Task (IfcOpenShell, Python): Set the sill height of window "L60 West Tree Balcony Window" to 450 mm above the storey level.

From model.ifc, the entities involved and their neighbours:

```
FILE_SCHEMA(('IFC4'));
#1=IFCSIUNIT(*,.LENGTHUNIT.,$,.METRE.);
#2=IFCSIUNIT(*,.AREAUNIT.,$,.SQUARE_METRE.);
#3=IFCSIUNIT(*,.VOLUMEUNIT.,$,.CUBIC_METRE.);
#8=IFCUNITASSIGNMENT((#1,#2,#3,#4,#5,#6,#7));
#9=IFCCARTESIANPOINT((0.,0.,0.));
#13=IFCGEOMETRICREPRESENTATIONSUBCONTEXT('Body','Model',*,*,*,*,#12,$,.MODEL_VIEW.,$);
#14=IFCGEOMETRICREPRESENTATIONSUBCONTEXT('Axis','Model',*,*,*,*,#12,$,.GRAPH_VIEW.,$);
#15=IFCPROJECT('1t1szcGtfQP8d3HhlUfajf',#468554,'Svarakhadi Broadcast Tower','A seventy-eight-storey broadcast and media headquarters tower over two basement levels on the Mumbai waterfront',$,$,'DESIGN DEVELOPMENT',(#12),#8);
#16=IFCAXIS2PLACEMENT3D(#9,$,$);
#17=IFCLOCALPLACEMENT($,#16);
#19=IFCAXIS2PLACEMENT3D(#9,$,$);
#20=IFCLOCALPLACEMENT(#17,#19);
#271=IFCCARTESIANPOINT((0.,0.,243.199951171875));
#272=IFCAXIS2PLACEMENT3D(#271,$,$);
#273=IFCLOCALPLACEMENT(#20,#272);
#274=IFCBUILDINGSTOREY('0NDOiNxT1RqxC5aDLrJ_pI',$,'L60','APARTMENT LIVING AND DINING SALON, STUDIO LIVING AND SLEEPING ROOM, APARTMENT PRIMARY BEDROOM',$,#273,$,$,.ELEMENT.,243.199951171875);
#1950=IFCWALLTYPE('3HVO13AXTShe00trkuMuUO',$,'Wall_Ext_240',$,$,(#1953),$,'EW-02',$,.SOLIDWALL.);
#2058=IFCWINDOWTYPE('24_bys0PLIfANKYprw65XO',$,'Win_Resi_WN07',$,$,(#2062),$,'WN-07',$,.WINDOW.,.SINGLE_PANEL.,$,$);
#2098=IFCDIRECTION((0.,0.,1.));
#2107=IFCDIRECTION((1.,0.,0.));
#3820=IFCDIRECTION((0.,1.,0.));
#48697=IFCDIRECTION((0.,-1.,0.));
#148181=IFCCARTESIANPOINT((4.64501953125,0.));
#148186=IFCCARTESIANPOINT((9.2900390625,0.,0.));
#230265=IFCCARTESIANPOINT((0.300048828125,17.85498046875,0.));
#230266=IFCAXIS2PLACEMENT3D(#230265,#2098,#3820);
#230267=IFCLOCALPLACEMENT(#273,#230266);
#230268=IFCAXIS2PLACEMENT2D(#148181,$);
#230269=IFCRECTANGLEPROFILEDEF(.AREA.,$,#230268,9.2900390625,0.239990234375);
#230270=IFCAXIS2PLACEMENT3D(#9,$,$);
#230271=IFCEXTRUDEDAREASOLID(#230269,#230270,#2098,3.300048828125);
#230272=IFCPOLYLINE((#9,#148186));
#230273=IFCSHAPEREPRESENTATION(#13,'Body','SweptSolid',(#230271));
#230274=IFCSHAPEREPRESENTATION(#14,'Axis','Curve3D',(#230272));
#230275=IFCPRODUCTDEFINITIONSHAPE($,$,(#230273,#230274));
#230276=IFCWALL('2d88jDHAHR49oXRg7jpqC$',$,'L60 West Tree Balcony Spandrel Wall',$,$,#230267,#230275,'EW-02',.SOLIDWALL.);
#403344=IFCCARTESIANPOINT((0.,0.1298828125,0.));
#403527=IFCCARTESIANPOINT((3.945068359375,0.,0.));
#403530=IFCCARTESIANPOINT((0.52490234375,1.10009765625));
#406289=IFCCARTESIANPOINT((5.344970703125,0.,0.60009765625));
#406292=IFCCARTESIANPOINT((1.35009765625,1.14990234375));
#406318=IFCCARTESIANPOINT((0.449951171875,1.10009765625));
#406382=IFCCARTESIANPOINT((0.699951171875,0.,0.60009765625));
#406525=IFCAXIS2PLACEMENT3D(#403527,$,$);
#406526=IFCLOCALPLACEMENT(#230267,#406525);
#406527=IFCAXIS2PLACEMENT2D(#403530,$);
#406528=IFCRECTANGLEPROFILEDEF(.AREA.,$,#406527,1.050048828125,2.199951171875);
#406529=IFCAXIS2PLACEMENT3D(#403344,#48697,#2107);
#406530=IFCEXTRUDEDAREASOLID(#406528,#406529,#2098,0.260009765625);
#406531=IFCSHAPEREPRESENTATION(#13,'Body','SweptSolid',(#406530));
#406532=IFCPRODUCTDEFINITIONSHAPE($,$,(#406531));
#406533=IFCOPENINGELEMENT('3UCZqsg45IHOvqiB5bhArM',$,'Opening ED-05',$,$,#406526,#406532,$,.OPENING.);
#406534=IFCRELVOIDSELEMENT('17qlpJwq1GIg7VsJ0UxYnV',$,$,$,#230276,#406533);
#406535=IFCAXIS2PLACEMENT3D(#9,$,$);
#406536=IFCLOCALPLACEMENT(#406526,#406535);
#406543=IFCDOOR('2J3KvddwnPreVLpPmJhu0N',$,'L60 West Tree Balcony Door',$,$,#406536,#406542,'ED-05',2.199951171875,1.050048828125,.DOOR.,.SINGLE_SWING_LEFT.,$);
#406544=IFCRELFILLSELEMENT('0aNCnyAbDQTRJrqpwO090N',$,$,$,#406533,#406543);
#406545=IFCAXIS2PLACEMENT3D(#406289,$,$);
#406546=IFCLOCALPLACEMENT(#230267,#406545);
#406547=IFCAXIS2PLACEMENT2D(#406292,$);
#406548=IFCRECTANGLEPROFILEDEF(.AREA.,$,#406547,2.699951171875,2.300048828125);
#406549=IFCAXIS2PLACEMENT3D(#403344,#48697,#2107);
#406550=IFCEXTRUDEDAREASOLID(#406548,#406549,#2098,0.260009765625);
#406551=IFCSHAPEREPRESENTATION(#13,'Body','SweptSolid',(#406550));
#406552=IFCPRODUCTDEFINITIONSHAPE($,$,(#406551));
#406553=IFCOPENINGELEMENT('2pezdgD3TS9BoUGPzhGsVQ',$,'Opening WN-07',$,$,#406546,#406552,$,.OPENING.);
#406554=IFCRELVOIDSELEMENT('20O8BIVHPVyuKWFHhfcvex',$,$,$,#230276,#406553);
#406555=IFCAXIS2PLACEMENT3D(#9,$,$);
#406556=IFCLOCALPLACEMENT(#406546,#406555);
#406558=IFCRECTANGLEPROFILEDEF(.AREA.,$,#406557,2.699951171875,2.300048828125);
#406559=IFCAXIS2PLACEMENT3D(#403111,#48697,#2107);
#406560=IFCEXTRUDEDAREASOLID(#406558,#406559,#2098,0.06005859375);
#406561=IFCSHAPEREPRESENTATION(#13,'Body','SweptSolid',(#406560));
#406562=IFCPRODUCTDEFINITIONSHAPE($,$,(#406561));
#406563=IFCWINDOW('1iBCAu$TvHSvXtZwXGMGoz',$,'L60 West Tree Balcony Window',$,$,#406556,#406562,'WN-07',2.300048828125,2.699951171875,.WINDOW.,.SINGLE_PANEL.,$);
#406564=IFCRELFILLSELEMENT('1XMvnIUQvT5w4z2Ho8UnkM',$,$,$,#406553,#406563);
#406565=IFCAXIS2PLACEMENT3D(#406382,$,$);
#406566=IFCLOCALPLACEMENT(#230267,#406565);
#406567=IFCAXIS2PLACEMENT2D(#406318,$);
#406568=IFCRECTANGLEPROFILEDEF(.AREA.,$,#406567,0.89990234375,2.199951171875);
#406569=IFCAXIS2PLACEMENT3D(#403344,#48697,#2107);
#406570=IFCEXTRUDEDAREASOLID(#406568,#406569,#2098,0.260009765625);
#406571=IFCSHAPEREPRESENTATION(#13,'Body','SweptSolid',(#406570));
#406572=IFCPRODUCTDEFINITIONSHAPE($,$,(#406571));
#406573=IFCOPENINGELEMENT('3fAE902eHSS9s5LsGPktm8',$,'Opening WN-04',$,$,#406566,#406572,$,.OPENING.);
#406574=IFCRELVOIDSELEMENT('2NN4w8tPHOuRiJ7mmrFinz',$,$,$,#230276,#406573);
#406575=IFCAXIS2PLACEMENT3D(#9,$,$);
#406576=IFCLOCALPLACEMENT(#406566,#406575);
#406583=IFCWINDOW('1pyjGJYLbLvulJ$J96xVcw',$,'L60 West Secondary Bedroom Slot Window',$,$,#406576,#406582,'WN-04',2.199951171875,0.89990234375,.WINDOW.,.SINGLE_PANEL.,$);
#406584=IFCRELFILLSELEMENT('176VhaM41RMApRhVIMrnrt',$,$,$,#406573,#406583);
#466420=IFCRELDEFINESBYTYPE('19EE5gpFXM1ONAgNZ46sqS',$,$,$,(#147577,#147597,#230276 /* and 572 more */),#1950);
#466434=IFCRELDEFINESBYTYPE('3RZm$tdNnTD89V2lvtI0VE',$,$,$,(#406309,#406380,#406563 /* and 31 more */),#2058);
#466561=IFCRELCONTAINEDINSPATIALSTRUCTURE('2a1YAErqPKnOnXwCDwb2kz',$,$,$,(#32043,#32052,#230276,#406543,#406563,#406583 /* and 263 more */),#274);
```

```python
import numpy as np
import ifcopenshell
import ifcopenshell.api.geometry
import ifcopenshell.geom
import ifcopenshell.util.element
import ifcopenshell.util.placement
import ifcopenshell.util.shape
import ifcopenshell.util.unit

model = ifcopenshell.open("model.ifc")
unit_scale = ifcopenshell.util.unit.calculate_unit_scale(model)

window = model.by_guid("1iBCAu$TvHSvXtZwXGMGoz")
opening = window.FillsVoids[0].RelatingOpeningElement
storey = ifcopenshell.util.element.get_container(window, ifc_class="IfcBuildingStorey")
level = ifcopenshell.util.placement.get_local_placement(storey.ObjectPlacement)[2, 3]

# The opening's origin need not be at the sill, so measure its lowest point.
shape = ifcopenshell.geom.create_shape(ifcopenshell.geom.settings(), opening)
bottom = ifcopenshell.util.shape.get_shape_bottom_elevation(shape, shape.geometry) / unit_scale
dz = level + 0.45 / unit_scale - bottom

shift = np.array([0.0, 0.0, dz])
# The window is placed relative to its opening, so it follows when the opening moves.
matrix = ifcopenshell.util.placement.get_local_placement(opening.ObjectPlacement)
matrix[:3, 3] += shift
ifcopenshell.api.geometry.edit_object_placement(
    model, product=opening, matrix=matrix, is_si=False, should_transform_children=True
)

print(f"moved by {dz * unit_scale:+.3f} m")

model.write("model_edited.ifc")
```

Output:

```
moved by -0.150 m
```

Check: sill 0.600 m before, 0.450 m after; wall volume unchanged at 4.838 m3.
